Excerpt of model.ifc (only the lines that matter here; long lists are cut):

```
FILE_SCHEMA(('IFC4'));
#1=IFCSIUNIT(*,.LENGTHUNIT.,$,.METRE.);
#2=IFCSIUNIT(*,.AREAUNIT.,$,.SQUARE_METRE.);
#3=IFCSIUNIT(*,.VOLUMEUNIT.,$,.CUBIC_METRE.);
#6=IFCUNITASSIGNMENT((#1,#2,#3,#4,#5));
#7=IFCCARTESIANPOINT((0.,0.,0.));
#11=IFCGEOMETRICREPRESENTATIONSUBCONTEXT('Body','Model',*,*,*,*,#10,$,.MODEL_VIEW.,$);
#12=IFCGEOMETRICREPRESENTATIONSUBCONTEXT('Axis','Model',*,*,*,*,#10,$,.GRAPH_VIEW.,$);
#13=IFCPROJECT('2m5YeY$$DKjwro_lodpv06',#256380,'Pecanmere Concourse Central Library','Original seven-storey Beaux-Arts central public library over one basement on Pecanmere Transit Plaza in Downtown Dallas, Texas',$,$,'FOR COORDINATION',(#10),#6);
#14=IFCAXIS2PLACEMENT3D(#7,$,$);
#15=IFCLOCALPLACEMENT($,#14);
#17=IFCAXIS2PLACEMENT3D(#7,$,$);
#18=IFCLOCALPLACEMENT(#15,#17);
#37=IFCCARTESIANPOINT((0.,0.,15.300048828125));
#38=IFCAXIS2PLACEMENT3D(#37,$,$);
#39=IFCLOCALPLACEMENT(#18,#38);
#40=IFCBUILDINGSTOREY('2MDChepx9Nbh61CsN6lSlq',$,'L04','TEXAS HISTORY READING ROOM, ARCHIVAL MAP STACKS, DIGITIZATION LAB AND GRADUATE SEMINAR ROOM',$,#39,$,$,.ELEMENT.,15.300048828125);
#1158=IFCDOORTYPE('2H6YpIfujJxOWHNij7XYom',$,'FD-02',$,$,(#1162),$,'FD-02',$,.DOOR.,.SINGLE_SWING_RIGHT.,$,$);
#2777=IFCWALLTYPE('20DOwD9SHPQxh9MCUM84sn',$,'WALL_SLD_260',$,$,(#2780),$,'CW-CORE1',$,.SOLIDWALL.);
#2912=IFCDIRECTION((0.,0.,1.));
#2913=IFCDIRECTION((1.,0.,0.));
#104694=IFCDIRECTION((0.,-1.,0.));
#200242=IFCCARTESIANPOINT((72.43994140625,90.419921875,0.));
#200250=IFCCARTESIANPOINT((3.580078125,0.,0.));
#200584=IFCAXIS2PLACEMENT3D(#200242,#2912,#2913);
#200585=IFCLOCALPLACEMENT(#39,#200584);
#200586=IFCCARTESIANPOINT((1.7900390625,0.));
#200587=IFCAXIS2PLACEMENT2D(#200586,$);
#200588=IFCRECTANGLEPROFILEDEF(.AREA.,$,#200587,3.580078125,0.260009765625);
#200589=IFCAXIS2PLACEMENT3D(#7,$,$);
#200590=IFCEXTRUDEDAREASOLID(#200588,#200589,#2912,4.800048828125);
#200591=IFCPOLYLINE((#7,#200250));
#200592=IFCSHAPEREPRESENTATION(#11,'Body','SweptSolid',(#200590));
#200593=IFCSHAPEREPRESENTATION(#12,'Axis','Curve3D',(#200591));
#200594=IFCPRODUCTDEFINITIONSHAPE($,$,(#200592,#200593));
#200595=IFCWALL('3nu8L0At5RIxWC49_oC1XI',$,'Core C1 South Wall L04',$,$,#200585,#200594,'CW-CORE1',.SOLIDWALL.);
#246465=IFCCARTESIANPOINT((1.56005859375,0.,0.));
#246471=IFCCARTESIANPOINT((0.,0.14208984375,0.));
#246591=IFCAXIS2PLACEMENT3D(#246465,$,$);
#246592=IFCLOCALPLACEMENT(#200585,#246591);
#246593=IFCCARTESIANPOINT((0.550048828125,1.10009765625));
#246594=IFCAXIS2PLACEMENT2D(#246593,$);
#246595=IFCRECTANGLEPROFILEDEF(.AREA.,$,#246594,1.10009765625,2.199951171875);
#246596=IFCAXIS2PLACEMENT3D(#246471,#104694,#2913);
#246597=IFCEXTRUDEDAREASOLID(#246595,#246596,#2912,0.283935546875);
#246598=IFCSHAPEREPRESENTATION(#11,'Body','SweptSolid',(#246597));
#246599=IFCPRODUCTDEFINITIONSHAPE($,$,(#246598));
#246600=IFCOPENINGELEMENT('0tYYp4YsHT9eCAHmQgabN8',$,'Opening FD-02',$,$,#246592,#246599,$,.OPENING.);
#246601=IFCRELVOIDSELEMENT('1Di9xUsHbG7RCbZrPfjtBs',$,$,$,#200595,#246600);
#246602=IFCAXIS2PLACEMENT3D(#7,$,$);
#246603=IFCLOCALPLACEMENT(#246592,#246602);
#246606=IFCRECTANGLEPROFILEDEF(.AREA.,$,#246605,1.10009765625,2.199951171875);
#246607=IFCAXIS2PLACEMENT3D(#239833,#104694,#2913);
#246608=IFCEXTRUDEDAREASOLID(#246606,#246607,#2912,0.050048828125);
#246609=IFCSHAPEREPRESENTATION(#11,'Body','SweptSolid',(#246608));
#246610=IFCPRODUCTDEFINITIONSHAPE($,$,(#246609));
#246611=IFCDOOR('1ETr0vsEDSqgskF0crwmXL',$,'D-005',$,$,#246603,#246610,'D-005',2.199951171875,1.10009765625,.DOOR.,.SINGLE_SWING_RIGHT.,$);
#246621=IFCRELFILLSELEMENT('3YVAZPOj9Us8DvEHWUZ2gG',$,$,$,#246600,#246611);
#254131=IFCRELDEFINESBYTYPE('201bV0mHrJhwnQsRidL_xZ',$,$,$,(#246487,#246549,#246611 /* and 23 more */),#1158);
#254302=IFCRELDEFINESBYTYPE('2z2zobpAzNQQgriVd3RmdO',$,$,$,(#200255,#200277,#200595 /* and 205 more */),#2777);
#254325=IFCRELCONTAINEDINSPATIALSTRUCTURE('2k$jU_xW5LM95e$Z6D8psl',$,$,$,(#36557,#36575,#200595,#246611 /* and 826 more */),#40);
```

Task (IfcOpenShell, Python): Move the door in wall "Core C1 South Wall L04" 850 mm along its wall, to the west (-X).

```python
import ifcopenshell
import ifcopenshell.api.geometry
import ifcopenshell.util.placement

model = ifcopenshell.open("model.ifc")

door = model.by_guid("1ETr0vsEDSqgskF0crwmXL")
opening = door.FillsVoids[0].RelatingOpeningElement
wall = opening.VoidsElements[0].RelatingBuildingElement

wall_matrix = ifcopenshell.util.placement.get_local_placement(wall.ObjectPlacement)
shift = wall_matrix[:3, 0] * -0.85
before = ifcopenshell.util.placement.get_local_placement(door.ObjectPlacement)[:3, 3].copy()

# The door is placed relative to its opening, so it follows when the opening moves.
matrix = ifcopenshell.util.placement.get_local_placement(opening.ObjectPlacement)
matrix[:3, 3] += shift
ifcopenshell.api.geometry.edit_object_placement(
    model, product=opening, matrix=matrix, is_si=False, should_transform_children=True
)

after = ifcopenshell.util.placement.get_local_placement(door.ObjectPlacement)[:3, 3]
print("door moved by", (after - before).round(3) + 0.0)

model.write("model_rev.ifc")
```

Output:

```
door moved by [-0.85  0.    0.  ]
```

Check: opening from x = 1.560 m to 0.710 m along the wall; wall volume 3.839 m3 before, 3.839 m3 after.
